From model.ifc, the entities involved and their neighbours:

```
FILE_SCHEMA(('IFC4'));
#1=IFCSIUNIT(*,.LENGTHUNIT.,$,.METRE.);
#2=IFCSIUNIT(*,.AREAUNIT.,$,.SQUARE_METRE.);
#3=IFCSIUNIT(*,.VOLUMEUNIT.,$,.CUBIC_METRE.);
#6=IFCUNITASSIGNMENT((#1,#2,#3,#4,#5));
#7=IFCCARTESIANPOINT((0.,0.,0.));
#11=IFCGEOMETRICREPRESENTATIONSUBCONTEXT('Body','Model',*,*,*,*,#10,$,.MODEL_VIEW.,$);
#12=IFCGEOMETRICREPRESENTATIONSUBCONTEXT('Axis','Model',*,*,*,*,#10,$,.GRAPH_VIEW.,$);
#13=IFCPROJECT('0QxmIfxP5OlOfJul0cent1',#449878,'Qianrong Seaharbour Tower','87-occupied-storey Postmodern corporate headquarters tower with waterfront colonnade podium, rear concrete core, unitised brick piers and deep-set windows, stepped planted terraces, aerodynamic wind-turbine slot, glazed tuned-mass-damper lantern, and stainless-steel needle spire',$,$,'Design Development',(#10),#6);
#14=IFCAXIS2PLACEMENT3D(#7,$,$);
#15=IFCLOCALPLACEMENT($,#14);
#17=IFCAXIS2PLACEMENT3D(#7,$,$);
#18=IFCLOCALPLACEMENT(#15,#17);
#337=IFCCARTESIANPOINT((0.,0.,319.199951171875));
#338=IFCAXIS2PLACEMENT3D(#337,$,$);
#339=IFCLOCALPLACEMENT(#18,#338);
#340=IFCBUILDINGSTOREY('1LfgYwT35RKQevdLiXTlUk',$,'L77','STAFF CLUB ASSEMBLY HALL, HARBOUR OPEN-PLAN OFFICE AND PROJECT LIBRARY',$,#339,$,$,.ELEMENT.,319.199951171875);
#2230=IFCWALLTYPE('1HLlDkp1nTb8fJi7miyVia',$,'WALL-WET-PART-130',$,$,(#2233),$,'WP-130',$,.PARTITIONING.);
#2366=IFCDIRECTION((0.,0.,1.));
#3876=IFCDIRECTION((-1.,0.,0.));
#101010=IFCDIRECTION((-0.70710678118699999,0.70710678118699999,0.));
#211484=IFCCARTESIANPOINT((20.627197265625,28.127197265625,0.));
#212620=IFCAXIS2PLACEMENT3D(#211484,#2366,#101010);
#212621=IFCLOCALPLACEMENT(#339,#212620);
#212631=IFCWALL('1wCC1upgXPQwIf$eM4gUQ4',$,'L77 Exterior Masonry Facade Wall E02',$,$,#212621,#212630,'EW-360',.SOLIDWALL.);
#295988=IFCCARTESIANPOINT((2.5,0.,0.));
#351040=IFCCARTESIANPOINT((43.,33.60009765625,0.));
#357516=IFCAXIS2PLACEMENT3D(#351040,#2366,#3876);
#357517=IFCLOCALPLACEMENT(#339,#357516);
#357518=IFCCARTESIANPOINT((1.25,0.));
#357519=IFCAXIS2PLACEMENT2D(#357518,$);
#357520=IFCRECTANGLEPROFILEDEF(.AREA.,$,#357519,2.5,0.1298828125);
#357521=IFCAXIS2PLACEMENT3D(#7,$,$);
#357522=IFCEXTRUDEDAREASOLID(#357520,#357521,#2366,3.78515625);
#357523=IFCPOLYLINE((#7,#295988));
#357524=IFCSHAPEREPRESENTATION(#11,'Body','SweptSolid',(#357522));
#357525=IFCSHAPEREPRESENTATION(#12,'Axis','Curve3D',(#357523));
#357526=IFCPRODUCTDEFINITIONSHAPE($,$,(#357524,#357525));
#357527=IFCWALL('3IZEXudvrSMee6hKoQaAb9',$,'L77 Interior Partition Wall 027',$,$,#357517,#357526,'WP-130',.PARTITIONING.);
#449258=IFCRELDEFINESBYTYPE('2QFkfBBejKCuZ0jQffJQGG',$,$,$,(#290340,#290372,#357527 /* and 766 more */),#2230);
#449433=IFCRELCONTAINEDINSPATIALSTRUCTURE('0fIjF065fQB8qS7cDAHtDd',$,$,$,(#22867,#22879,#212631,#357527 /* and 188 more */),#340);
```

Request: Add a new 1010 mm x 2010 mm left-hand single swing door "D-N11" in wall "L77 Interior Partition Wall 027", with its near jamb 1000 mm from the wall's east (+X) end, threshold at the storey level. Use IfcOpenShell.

```python
import numpy as np
import ifcopenshell
import ifcopenshell.api.feature
import ifcopenshell.api.geometry
import ifcopenshell.api.root
import ifcopenshell.api.spatial
import ifcopenshell.geom
import ifcopenshell.util.element
import ifcopenshell.util.placement
import ifcopenshell.util.representation
import ifcopenshell.util.shape
import ifcopenshell.util.unit

model = ifcopenshell.open("model.ifc")
unit_scale = ifcopenshell.util.unit.calculate_unit_scale(model)
settings = ifcopenshell.geom.settings()


def volume(element):
    """Net volume in cubic metres, openings subtracted."""
    shape = ifcopenshell.geom.create_shape(settings, element)
    return ifcopenshell.util.shape.get_volume(shape.geometry)


wall = model.by_id(357527)
storey = ifcopenshell.util.element.get_container(wall, ifc_class="IfcBuildingStorey")
context = ifcopenshell.util.representation.get_context(model, "Model", "Body", "MODEL_VIEW")
before = volume(wall)

width, height, from_end, sill = 1.01, 2.01, 1, 0.0  # metres

# The wall runs along its own X axis, and the end named is its -X end.
wall_shape = ifcopenshell.geom.create_shape(settings, wall)
x, y, z = ifcopenshell.util.shape.get_vertices(wall_shape.geometry).T
start = x.min() + from_end
face, thickness = float(y.min()), float(y.max() - y.min())
wall_matrix = ifcopenshell.util.placement.get_local_placement(wall.ObjectPlacement)
level = ifcopenshell.util.placement.get_local_placement(storey.ObjectPlacement)[2, 3]


def in_wall(x, y):
    """Placement at x, y metres in the wall's axes, at sill height."""
    matrix = wall_matrix.copy()
    matrix[:, 3] = wall_matrix @ np.array([x / unit_scale, y / unit_scale, 0.0, 1.0])
    matrix[2, 3] = level + sill / unit_scale
    return matrix


# Opening: a box that overshoots both wall faces by 50 mm.
opening = ifcopenshell.api.root.create_entity(model, ifc_class="IfcOpeningElement", predefined_type="OPENING")
box = ifcopenshell.api.geometry.add_wall_representation(
    model, context=context, length=width, height=height, thickness=thickness + 0.1
)
ifcopenshell.api.geometry.assign_representation(model, product=opening, representation=box)
ifcopenshell.api.geometry.edit_object_placement(model, product=opening, matrix=in_wall(start, face - 0.05), is_si=False)
ifcopenshell.api.feature.add_feature(model, feature=opening, element=wall)

door = ifcopenshell.api.root.create_entity(model, ifc_class="IfcDoor", name="D-N11", predefined_type="DOOR")
door.OverallWidth, door.OverallHeight = width / unit_scale, height / unit_scale
door.OperationType = "SINGLE_SWING_LEFT"
body = ifcopenshell.api.geometry.add_door_representation(
    model,
    context=context,
    overall_width=door.OverallWidth,
    overall_height=door.OverallHeight,
    operation_type="SINGLE_SWING_LEFT",
    lining_properties={"LiningDepth": thickness / unit_scale, "ThresholdDepth": thickness / unit_scale},
)
ifcopenshell.api.geometry.assign_representation(model, product=door, representation=body)
ifcopenshell.api.spatial.assign_container(model, products=[door], relating_structure=storey)
ifcopenshell.api.feature.add_filling(model, opening=opening, element=door)

# The lining spans the wall, so the door starts at the wall face.
ifcopenshell.api.geometry.edit_object_placement(model, product=door, matrix=in_wall(start, face), is_si=False)

after = volume(wall)

print(f"wall volume {before:.3f} -> {after:.3f} m3")

model.write("model_rev.ifc")
```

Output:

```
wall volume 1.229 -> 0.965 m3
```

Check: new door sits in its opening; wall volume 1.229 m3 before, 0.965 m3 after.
